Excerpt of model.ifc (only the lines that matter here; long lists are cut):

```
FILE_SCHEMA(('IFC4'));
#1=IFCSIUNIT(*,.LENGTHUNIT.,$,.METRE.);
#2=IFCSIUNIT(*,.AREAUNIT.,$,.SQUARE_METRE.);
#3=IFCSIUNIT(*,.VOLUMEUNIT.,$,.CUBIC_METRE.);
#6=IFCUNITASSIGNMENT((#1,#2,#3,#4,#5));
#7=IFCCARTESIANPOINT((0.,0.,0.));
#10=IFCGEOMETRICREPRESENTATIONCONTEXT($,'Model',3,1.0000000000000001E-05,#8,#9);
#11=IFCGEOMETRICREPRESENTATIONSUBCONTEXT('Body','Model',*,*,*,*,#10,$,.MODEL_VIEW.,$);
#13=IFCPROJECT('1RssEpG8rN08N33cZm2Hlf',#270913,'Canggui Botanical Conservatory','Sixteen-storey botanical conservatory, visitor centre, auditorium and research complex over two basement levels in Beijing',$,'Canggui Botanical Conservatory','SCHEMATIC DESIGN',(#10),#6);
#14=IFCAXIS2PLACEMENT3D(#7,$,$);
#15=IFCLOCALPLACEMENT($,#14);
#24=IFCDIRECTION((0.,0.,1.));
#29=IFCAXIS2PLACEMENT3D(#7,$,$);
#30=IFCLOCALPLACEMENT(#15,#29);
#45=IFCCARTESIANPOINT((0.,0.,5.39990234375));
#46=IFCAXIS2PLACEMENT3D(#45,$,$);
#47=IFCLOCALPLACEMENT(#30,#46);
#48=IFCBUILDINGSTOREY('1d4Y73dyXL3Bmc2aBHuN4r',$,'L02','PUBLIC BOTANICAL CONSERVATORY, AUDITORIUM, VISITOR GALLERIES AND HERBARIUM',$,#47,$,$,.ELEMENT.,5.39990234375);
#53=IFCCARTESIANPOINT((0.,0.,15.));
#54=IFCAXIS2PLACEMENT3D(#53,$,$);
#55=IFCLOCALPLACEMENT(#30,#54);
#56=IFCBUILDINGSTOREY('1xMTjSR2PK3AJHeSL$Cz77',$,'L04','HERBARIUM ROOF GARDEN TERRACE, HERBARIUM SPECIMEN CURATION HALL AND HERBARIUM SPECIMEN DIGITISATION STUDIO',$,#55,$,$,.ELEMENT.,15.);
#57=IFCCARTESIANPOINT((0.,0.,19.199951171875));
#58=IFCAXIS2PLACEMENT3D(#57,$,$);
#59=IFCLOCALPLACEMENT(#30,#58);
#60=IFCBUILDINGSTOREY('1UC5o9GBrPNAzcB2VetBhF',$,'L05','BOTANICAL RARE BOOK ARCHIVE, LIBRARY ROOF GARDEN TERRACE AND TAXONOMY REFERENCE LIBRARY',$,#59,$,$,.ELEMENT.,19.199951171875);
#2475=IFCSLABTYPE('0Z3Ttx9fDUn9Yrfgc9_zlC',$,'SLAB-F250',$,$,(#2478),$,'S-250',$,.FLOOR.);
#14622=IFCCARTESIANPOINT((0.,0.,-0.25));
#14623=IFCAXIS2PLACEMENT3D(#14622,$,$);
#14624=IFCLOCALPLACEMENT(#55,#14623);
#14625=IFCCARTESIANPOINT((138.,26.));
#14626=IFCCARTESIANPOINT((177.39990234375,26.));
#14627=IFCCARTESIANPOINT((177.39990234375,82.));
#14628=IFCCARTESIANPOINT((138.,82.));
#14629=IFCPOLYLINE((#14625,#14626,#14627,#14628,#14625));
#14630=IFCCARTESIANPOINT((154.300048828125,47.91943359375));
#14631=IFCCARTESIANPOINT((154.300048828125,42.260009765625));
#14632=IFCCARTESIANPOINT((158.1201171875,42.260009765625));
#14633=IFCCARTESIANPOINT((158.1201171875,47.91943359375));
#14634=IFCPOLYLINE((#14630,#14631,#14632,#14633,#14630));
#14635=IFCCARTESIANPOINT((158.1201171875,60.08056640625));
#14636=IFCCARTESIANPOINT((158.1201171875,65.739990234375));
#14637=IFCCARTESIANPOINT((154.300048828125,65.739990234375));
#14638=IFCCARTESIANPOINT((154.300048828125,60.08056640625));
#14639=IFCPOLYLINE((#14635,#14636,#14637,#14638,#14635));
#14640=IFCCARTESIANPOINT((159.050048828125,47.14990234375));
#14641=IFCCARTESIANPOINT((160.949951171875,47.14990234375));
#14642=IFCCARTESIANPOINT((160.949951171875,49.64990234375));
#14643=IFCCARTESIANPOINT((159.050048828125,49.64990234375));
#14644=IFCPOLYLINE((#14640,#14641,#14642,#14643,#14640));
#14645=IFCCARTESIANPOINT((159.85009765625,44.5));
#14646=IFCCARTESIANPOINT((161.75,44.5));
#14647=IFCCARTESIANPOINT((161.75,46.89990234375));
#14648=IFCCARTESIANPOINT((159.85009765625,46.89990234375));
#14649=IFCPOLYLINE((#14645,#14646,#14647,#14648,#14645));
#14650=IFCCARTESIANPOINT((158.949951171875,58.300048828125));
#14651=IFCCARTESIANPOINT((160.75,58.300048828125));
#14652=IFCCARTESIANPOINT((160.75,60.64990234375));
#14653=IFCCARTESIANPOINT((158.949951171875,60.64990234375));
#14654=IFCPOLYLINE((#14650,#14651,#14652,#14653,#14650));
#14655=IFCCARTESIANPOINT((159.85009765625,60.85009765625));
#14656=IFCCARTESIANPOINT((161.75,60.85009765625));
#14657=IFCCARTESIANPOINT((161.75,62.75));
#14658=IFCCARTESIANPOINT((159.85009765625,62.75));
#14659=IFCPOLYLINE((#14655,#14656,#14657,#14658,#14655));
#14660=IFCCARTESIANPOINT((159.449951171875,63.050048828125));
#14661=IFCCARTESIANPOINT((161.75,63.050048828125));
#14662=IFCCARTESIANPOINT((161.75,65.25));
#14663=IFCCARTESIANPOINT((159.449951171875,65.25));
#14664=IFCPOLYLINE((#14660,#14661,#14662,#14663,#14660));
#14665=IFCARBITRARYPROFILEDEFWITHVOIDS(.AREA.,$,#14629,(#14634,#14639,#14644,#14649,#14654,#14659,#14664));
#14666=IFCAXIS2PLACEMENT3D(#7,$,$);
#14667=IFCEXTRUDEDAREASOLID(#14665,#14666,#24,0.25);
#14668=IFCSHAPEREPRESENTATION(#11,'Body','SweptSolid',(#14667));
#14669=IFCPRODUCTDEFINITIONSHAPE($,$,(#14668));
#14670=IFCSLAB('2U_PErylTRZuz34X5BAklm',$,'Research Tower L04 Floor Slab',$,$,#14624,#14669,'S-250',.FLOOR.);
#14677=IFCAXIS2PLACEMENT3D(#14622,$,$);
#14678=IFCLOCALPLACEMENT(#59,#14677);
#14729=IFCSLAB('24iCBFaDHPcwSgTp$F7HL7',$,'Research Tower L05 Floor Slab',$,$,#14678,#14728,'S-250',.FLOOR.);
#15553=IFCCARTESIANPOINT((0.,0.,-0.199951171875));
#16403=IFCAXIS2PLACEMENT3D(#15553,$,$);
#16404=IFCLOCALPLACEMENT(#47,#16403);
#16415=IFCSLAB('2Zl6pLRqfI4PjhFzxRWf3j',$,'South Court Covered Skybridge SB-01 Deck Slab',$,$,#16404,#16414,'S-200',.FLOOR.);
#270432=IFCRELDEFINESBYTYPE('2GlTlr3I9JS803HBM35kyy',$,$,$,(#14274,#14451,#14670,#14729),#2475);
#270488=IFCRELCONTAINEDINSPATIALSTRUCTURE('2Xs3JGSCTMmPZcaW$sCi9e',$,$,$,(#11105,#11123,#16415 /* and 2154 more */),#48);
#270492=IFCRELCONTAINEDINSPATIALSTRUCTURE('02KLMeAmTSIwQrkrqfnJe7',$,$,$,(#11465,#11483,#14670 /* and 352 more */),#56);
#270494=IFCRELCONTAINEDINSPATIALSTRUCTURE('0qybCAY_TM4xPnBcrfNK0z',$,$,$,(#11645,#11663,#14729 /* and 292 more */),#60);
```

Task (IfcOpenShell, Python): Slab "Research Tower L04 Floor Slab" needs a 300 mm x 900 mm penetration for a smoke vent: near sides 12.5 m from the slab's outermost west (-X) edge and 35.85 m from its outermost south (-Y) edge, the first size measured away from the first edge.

```python
import numpy as np
import ifcopenshell
import ifcopenshell.api.feature
import ifcopenshell.api.geometry
import ifcopenshell.api.root
import ifcopenshell.geom
import ifcopenshell.util.placement
import ifcopenshell.util.representation
import ifcopenshell.util.shape
import ifcopenshell.util.unit

model = ifcopenshell.open("model.ifc")
unit_scale = ifcopenshell.util.unit.calculate_unit_scale(model)
settings = ifcopenshell.geom.settings()


def volume(element):
    """Net volume in cubic metres, openings subtracted."""
    shape = ifcopenshell.geom.create_shape(settings, element)
    return ifcopenshell.util.shape.get_volume(shape.geometry)


slab = model.by_guid("2U_PErylTRZuz34X5BAklm")
before = volume(slab)

# Extent in the slab's own axes, in metres. The edges named are its -X and -Y sides.
slab_shape = ifcopenshell.geom.create_shape(settings, slab)
vertices = ifcopenshell.util.shape.get_vertices(slab_shape.geometry)
x_min, y_min, bottom = vertices.min(axis=0)
top = vertices[:, 2].max()

opening = ifcopenshell.api.root.create_entity(model, ifc_class="IfcOpeningElement", name="Smoke vent opening", predefined_type="OPENING")
context = ifcopenshell.util.representation.get_context(model, "Model", "Body", "MODEL_VIEW")
width, depth = 0.3, 0.9
outline = [(0.0, 0.0), (width, 0.0), (width, depth), (0.0, depth), (0.0, 0.0)]
# Overshoot both faces by 50 mm so the cut is clean.
shape = ifcopenshell.api.geometry.add_slab_representation(
    model, context=context, depth=top - bottom + 0.1, polyline=outline
)
ifcopenshell.api.geometry.assign_representation(model, product=opening, representation=shape)

matrix = ifcopenshell.util.placement.get_local_placement(slab.ObjectPlacement)
matrix[:, 3] = matrix @ np.append(np.array([x_min + 12.5, y_min + 35.85, bottom - 0.05]) / unit_scale, 1.0)
ifcopenshell.api.geometry.edit_object_placement(model, product=opening, matrix=matrix, is_si=False)
ifcopenshell.api.feature.add_feature(model, feature=opening, element=slab)

after = volume(slab)

print(f"slab volume {before:.3f} -> {after:.3f} m3")

model.write("model-out.ifc")
```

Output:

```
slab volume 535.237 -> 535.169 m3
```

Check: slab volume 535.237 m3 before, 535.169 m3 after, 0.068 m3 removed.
